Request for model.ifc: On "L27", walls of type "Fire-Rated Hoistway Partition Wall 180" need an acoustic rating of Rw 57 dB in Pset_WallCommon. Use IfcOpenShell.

First a look at what the model holds.

```python
import ifcopenshell
import ifcopenshell.util.element

model = ifcopenshell.open("model.ifc")
print(model.schema)
storey = next(s for s in model.by_type("IfcBuildingStorey") if s.Name == "L27")
walls = [e for e in ifcopenshell.util.element.get_decomposition(storey) if e.is_a("IfcWall")]
seen = {}
for e in walls:
    element_type = ifcopenshell.util.element.get_type(e)
    key = (element_type.Name if element_type != e and element_type else None, ifcopenshell.util.element.get_pset(e, "Pset_WallCommon", "AcousticRating"))
    seen[key] = seen.get(key, 0) + 1
for (name, value), count in sorted(seen.items(), key=str):
    print(count, "x", name, "|", value)
```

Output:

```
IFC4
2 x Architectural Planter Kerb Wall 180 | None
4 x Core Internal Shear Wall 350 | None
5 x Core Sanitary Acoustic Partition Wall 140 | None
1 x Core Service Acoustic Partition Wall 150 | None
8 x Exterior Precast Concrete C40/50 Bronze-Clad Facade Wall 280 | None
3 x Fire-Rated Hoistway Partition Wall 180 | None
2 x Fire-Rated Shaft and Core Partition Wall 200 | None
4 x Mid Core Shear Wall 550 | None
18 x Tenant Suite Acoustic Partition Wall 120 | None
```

```python
import ifcopenshell
import ifcopenshell.api.pset
import ifcopenshell.util.element

model = ifcopenshell.open("model.ifc")

storey = next(s for s in model.by_type("IfcBuildingStorey") if s.Name == "L27")
walls = [e for e in ifcopenshell.util.element.get_decomposition(storey) if e.is_a("IfcWall")]

count = 0
for e in walls:
    element_type = ifcopenshell.util.element.get_type(e)
    if element_type in (None, e) or element_type.Name != "Fire-Rated Hoistway Partition Wall 180":
        continue
    # add_pset returns the element's existing set when there is one.
    pset = ifcopenshell.api.pset.add_pset(model, product=e, name="Pset_WallCommon")
    ifcopenshell.api.pset.edit_pset(model, pset=pset, properties={"AcousticRating": "Rw 57 dB"})
    count += 1

print(count, "walls updated")

model.write("model-out.ifc")
```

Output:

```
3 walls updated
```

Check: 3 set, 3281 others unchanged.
